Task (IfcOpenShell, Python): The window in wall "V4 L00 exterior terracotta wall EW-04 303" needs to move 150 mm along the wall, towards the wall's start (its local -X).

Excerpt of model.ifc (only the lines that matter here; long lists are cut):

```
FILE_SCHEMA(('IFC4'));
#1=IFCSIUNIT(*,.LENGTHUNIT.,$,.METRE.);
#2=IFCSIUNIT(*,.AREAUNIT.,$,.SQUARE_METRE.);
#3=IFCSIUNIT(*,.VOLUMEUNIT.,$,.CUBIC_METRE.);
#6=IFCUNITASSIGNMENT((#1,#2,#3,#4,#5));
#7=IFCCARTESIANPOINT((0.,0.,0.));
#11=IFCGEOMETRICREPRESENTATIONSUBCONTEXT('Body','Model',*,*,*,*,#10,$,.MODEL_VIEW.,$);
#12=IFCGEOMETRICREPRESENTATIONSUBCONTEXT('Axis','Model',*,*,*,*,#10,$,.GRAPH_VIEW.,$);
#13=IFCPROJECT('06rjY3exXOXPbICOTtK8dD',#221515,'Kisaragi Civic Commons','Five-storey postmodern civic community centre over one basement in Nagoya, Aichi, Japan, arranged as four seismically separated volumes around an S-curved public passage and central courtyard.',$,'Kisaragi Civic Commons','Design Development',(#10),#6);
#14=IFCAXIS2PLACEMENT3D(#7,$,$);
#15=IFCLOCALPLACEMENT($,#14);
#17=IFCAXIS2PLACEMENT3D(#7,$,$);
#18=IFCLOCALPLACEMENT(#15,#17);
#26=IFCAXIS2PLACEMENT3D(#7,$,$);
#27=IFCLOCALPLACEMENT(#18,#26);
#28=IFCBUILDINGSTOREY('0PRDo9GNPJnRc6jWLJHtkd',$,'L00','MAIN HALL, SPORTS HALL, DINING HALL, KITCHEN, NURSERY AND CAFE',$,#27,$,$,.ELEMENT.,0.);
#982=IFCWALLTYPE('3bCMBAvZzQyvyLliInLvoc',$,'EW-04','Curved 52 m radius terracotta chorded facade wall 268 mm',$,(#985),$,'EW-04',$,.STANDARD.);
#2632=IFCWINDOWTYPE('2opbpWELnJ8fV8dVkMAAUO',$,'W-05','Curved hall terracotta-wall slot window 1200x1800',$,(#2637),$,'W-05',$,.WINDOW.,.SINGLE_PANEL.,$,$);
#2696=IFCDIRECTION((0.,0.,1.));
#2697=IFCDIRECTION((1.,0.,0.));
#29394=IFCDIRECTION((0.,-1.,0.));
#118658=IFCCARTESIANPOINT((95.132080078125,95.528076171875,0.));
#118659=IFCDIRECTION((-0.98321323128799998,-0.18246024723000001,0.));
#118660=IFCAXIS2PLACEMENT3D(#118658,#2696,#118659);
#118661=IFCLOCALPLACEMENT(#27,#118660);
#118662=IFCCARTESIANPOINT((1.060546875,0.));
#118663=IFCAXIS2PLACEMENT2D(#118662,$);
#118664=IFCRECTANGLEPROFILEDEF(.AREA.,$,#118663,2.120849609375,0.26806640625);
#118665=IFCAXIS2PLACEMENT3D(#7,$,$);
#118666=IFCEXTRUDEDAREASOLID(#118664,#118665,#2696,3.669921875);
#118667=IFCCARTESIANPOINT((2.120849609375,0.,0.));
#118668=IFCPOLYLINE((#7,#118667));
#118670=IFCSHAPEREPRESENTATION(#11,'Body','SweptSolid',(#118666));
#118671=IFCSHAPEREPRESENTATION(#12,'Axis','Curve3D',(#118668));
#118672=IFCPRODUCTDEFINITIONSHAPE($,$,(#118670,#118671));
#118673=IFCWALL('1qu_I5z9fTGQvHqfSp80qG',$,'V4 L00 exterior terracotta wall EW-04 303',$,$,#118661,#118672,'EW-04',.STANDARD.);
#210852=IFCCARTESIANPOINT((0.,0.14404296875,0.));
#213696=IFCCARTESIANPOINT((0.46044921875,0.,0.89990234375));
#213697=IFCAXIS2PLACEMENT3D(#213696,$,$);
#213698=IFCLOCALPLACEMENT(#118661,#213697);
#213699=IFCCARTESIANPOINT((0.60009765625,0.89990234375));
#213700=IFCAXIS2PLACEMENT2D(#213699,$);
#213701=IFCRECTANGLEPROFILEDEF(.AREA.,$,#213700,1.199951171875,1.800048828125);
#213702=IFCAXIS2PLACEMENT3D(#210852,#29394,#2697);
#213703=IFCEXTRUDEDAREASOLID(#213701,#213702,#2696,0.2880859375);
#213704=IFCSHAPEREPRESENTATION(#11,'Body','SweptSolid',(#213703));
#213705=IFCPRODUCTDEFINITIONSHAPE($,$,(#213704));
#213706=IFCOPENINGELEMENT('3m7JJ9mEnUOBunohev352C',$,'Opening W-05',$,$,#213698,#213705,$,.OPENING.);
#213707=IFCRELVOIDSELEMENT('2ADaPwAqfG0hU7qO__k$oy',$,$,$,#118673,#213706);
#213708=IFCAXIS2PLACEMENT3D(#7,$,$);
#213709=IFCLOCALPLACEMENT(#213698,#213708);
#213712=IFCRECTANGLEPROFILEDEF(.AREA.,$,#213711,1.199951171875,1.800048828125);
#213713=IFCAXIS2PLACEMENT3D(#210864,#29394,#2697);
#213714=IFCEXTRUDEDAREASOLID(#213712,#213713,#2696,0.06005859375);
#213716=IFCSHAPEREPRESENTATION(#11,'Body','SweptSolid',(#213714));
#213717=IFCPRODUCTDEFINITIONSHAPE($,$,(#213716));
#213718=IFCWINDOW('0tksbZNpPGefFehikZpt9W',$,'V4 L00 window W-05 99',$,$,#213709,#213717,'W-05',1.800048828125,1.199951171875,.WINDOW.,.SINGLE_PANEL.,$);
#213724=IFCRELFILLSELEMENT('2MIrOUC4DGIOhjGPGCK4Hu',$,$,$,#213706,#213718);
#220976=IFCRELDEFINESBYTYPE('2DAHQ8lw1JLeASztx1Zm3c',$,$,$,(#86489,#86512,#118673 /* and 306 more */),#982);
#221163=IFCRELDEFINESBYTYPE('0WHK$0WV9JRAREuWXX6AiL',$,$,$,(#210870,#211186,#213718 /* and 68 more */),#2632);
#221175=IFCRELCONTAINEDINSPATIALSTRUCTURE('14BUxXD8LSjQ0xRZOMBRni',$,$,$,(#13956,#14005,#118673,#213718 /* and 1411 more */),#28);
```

```python
import ifcopenshell
import ifcopenshell.api.geometry
import ifcopenshell.util.placement
import ifcopenshell.util.unit

model = ifcopenshell.open("model.ifc")
unit_scale = ifcopenshell.util.unit.calculate_unit_scale(model)

window = model.by_guid("0tksbZNpPGefFehikZpt9W")
opening = window.FillsVoids[0].RelatingOpeningElement
wall = opening.VoidsElements[0].RelatingBuildingElement

wall_matrix = ifcopenshell.util.placement.get_local_placement(wall.ObjectPlacement)
shift = wall_matrix[:3, 0] * -0.15 / unit_scale
before = ifcopenshell.util.placement.get_local_placement(window.ObjectPlacement)[:3, 3].copy()

# The window is placed relative to its opening, so it follows when the opening moves.
matrix = ifcopenshell.util.placement.get_local_placement(opening.ObjectPlacement)
matrix[:3, 3] += shift
ifcopenshell.api.geometry.edit_object_placement(
    model, product=opening, matrix=matrix, is_si=False, should_transform_children=True
)

after = ifcopenshell.util.placement.get_local_placement(window.ObjectPlacement)[:3, 3]
print("window moved by", (after - before).round(3) + 0.0)

model.write("model-out.ifc")
```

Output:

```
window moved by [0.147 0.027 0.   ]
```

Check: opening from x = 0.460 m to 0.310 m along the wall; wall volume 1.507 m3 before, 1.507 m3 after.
